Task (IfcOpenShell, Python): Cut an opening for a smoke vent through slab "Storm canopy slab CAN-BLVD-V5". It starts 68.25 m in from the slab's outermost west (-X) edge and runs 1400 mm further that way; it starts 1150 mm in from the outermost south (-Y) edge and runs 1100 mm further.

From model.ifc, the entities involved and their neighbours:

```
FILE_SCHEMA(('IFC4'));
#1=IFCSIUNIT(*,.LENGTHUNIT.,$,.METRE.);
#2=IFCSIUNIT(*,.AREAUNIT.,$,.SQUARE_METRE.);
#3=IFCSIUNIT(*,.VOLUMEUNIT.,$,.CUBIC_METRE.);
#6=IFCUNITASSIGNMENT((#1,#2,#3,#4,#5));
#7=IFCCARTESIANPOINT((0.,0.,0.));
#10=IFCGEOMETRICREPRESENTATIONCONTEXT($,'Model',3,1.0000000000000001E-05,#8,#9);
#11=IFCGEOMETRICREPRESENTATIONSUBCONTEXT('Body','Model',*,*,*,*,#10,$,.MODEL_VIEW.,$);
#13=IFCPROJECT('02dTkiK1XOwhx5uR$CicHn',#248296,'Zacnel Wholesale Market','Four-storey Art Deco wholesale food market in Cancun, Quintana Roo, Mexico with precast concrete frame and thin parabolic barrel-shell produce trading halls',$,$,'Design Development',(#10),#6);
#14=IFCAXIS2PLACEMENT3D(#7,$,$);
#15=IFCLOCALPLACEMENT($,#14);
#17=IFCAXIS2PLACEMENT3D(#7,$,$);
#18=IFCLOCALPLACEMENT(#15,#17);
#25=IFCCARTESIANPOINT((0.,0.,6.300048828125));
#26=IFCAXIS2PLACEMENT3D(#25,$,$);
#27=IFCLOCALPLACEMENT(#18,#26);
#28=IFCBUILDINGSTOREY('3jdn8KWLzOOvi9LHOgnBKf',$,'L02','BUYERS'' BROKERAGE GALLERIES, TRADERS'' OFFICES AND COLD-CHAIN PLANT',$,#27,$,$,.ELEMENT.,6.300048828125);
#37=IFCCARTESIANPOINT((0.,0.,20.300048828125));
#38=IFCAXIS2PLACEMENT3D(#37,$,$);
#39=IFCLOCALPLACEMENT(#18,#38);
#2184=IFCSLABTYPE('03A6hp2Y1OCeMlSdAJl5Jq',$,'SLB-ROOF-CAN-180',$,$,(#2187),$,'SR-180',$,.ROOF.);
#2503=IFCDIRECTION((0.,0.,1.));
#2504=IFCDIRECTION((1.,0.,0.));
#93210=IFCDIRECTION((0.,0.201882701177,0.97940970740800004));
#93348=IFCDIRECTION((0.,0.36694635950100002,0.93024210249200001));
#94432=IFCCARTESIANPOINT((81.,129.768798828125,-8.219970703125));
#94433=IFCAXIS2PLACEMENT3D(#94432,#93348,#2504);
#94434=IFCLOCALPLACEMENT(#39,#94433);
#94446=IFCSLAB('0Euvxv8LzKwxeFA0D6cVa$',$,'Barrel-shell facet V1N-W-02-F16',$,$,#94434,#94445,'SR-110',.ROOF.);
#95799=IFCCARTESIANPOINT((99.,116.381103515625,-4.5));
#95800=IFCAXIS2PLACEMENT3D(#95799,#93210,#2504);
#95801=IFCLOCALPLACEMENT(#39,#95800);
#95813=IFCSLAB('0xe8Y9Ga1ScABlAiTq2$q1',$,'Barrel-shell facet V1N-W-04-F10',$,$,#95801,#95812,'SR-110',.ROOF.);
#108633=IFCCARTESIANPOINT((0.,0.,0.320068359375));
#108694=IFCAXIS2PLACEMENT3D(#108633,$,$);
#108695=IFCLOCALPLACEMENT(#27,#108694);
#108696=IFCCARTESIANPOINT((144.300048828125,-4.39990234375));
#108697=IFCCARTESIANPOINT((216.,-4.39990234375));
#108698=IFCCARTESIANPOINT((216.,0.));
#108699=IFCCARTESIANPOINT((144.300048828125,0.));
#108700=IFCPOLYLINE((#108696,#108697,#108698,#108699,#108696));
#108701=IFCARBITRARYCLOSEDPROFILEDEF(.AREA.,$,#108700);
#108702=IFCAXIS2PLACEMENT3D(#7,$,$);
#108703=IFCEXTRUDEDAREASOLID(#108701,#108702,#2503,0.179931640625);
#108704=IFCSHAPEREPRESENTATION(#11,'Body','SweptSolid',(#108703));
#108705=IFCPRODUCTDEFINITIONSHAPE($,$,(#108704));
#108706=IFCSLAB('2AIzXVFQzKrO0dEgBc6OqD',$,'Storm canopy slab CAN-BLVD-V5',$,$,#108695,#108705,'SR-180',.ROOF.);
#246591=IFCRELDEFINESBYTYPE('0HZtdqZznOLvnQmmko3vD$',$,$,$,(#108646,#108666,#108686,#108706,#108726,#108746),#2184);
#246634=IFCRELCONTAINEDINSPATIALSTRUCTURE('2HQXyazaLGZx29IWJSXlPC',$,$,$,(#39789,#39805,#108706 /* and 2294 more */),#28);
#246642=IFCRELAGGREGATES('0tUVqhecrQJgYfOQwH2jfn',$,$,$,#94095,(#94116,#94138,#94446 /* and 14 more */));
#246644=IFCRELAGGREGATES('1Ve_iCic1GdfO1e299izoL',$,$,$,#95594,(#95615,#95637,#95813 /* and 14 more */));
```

```python
import numpy as np
import ifcopenshell
import ifcopenshell.api.feature
import ifcopenshell.api.geometry
import ifcopenshell.api.root
import ifcopenshell.geom
import ifcopenshell.util.placement
import ifcopenshell.util.representation
import ifcopenshell.util.shape
import ifcopenshell.util.unit

model = ifcopenshell.open("model.ifc")
unit_scale = ifcopenshell.util.unit.calculate_unit_scale(model)
settings = ifcopenshell.geom.settings()


def volume(element):
    """Net volume in cubic metres, openings subtracted."""
    shape = ifcopenshell.geom.create_shape(settings, element)
    return ifcopenshell.util.shape.get_volume(shape.geometry)


slab = model.by_guid("2AIzXVFQzKrO0dEgBc6OqD")
before = volume(slab)

# Extent in the slab's own axes, in metres. The edges named are its -X and -Y sides.
slab_shape = ifcopenshell.geom.create_shape(settings, slab)
vertices = ifcopenshell.util.shape.get_vertices(slab_shape.geometry)
x_min, y_min, bottom = vertices.min(axis=0)
top = vertices[:, 2].max()

opening = ifcopenshell.api.root.create_entity(model, ifc_class="IfcOpeningElement", name="Smoke vent opening", predefined_type="OPENING")
context = ifcopenshell.util.representation.get_context(model, "Model", "Body", "MODEL_VIEW")
width, depth = 1.4, 1.1
outline = [(0.0, 0.0), (width, 0.0), (width, depth), (0.0, depth), (0.0, 0.0)]
# Overshoot both faces by 50 mm so the cut is clean.
shape = ifcopenshell.api.geometry.add_slab_representation(
    model, context=context, depth=top - bottom + 0.1, polyline=outline
)
ifcopenshell.api.geometry.assign_representation(model, product=opening, representation=shape)

matrix = ifcopenshell.util.placement.get_local_placement(slab.ObjectPlacement)
matrix[:, 3] = matrix @ np.append(np.array([x_min + 68.25, y_min + 1.15, bottom - 0.05]) / unit_scale, 1.0)
ifcopenshell.api.geometry.edit_object_placement(model, product=opening, matrix=matrix, is_si=False)
ifcopenshell.api.feature.add_feature(model, feature=opening, element=slab)

after = volume(slab)

print(f"slab volume {before:.3f} -> {after:.3f} m3")

model.write("model_v2.ifc")
```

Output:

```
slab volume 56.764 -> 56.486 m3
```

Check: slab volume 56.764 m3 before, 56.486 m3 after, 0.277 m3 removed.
